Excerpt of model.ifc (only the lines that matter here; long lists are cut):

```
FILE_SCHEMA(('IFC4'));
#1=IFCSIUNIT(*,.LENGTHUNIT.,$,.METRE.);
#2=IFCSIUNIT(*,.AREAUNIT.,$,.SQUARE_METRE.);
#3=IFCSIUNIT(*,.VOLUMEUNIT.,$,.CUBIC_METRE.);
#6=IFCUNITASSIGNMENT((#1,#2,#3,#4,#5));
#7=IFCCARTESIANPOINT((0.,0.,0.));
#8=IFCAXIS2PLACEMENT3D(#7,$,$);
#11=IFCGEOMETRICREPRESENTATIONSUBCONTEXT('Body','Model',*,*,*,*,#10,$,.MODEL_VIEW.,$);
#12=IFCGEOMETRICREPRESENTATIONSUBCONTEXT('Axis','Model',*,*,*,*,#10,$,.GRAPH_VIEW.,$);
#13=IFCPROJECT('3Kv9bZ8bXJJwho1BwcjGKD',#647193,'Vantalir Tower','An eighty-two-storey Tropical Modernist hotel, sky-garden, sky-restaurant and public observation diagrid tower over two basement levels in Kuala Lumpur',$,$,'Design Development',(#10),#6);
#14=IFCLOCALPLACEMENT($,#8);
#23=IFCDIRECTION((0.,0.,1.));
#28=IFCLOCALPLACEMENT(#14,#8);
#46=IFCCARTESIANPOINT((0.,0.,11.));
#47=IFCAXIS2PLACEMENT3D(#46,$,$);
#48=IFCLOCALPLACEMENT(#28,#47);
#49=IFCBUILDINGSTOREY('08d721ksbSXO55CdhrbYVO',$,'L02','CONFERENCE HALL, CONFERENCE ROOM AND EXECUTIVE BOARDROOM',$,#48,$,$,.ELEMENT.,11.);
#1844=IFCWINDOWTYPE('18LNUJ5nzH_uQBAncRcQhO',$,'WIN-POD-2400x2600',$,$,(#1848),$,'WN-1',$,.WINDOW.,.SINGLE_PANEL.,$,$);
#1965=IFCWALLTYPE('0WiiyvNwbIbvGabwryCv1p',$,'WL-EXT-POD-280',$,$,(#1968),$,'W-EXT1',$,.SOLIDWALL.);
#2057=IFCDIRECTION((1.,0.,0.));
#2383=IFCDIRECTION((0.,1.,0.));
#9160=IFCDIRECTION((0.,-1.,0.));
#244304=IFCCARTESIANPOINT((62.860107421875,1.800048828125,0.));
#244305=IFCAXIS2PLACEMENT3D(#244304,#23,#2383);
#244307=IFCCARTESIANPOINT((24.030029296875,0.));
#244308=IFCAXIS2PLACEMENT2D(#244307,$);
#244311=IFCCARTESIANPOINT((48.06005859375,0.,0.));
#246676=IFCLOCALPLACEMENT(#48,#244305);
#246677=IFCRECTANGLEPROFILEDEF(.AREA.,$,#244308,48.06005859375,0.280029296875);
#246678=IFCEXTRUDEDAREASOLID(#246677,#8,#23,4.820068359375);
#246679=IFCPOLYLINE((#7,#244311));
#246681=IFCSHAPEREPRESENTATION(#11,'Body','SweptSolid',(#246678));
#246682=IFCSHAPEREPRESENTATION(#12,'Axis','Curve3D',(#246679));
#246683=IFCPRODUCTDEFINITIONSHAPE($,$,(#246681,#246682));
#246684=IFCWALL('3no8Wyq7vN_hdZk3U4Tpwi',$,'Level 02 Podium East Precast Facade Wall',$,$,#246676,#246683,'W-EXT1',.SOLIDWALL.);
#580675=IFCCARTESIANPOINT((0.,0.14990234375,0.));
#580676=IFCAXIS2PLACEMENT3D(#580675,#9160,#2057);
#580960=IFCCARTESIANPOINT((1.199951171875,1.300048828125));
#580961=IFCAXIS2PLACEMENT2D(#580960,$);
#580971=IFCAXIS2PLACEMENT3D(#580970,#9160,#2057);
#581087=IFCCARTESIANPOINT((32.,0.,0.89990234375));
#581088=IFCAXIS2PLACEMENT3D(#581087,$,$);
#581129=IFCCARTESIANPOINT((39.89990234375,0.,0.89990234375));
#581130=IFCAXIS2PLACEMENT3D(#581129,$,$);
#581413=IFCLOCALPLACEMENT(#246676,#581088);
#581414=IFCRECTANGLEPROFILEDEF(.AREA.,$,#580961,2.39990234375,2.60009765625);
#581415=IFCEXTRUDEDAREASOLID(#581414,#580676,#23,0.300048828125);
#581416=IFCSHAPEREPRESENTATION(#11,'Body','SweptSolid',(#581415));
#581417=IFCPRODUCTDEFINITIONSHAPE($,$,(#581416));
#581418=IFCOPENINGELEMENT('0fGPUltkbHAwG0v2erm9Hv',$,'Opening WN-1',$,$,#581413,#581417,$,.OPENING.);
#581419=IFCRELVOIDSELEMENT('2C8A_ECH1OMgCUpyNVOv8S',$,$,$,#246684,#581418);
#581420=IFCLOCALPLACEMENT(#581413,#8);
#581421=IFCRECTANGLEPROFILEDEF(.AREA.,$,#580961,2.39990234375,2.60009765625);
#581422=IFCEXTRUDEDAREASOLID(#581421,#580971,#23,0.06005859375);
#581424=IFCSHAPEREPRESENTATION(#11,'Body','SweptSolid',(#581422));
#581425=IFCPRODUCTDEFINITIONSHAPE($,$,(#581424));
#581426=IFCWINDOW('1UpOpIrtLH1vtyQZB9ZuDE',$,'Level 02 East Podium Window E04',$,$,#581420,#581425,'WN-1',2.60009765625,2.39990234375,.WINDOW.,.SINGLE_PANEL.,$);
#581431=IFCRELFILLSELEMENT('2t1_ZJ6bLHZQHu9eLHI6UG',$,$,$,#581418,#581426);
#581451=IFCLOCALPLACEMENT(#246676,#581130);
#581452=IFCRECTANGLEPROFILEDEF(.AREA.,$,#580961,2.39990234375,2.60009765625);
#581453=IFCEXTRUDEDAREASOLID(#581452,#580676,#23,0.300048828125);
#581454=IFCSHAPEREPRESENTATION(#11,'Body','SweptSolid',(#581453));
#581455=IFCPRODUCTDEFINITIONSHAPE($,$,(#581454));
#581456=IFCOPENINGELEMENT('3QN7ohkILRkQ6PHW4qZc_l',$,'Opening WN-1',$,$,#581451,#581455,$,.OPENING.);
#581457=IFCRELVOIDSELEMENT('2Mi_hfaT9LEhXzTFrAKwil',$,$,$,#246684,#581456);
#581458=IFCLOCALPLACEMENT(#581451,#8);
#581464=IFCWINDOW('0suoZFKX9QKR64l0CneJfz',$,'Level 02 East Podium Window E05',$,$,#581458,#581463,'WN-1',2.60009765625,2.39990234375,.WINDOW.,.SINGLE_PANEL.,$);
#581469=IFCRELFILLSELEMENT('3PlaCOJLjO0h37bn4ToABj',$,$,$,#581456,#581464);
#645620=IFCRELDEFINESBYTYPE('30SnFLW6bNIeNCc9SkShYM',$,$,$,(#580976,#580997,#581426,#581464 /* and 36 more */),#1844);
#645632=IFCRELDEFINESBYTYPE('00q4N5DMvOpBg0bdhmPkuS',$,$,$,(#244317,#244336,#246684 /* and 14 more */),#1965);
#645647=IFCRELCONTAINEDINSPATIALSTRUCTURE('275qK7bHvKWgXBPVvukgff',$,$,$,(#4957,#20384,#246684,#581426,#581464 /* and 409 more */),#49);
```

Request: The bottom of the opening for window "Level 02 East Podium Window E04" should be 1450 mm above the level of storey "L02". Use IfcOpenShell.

```python
import numpy as np
import ifcopenshell
import ifcopenshell.api.geometry
import ifcopenshell.geom
import ifcopenshell.util.element
import ifcopenshell.util.placement
import ifcopenshell.util.shape
import ifcopenshell.util.unit

model = ifcopenshell.open("model.ifc")
unit_scale = ifcopenshell.util.unit.calculate_unit_scale(model)

window = model.by_guid("1UpOpIrtLH1vtyQZB9ZuDE")
opening = window.FillsVoids[0].RelatingOpeningElement
storey = ifcopenshell.util.element.get_container(window, ifc_class="IfcBuildingStorey")
level = ifcopenshell.util.placement.get_local_placement(storey.ObjectPlacement)[2, 3]

# The opening's origin need not be at the sill, so measure its lowest point.
shape = ifcopenshell.geom.create_shape(ifcopenshell.geom.settings(), opening)
bottom = ifcopenshell.util.shape.get_shape_bottom_elevation(shape, shape.geometry) / unit_scale
dz = level + 1.45 / unit_scale - bottom

shift = np.array([0.0, 0.0, dz])
# The window is placed relative to its opening, so it follows when the opening moves.
matrix = ifcopenshell.util.placement.get_local_placement(opening.ObjectPlacement)
matrix[:3, 3] += shift
ifcopenshell.api.geometry.edit_object_placement(
    model, product=opening, matrix=matrix, is_si=False, should_transform_children=True
)

print(f"moved by {dz * unit_scale:+.3f} m")

model.write("model_v2.ifc")
```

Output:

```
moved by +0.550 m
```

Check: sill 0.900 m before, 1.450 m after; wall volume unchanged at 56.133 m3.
